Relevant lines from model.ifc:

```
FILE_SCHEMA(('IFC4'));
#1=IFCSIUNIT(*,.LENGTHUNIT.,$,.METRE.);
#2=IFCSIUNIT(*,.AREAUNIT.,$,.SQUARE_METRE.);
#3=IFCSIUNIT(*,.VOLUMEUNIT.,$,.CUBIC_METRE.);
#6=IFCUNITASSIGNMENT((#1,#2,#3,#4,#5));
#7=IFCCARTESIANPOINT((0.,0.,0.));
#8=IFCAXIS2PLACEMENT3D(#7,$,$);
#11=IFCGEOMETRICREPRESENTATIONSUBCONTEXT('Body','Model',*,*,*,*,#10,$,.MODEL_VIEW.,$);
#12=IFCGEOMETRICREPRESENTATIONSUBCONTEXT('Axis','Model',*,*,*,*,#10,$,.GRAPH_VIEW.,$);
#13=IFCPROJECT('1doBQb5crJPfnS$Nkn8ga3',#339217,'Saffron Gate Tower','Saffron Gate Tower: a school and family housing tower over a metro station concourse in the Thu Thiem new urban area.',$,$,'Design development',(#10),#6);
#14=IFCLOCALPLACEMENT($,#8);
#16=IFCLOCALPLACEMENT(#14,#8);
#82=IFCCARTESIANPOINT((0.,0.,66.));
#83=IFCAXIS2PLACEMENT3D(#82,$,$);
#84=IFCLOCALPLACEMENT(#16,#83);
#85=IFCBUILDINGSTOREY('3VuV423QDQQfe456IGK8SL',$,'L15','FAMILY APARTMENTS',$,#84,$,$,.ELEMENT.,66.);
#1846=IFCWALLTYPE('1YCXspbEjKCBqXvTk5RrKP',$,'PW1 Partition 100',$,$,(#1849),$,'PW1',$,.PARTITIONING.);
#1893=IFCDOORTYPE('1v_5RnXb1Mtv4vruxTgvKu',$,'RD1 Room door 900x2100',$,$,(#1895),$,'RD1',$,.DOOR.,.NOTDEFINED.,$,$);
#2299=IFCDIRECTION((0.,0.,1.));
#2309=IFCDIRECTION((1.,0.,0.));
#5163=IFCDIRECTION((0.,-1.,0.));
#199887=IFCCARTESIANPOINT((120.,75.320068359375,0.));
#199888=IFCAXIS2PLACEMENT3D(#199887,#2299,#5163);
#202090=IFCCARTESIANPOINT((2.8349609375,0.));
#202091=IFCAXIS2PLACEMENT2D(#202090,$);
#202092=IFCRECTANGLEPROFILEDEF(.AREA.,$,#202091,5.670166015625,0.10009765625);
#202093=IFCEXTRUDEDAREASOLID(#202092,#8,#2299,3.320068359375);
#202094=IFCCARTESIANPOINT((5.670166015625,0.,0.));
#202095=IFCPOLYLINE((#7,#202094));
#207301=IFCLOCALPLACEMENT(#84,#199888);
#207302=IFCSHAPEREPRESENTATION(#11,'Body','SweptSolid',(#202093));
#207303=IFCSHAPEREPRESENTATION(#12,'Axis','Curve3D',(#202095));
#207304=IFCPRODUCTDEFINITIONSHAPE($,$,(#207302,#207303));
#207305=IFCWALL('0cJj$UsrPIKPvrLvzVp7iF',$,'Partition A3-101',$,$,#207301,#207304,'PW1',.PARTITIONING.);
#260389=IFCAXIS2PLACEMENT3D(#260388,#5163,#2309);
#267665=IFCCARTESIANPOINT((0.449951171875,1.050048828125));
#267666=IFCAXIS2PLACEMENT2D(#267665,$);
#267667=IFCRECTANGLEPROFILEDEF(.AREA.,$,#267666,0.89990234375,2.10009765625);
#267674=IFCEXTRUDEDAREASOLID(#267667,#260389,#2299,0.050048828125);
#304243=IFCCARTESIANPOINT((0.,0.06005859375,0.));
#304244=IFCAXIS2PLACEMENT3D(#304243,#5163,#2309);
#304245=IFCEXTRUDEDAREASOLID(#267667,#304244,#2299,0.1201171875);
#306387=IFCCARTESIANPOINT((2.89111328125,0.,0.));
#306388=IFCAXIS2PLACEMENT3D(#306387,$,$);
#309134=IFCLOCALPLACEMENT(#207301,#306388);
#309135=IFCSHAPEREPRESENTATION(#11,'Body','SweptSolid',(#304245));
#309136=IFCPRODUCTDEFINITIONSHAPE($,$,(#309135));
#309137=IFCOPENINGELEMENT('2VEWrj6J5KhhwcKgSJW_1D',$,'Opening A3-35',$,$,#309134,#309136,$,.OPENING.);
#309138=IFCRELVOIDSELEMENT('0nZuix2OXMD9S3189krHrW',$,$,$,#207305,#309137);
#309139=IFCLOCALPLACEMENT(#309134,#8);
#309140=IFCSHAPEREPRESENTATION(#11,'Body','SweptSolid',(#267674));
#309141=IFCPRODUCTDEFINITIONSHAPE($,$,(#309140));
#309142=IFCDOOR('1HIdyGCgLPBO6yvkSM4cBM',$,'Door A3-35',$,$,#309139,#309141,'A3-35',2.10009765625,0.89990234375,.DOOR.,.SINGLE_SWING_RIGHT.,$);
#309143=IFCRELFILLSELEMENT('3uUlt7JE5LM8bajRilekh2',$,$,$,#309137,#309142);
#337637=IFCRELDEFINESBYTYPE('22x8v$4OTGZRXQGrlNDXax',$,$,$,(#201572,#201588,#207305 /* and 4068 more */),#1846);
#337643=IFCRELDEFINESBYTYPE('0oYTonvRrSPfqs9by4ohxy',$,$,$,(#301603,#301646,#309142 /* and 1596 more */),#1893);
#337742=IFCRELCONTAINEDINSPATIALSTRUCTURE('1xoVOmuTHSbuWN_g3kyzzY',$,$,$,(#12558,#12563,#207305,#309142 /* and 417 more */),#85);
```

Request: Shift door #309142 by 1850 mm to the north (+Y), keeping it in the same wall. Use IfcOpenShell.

```python
import ifcopenshell
import ifcopenshell.api.geometry
import ifcopenshell.util.placement
import ifcopenshell.util.unit

model = ifcopenshell.open("model.ifc")
unit_scale = ifcopenshell.util.unit.calculate_unit_scale(model)

door = model.by_id(309142)
opening = door.FillsVoids[0].RelatingOpeningElement
wall = opening.VoidsElements[0].RelatingBuildingElement

wall_matrix = ifcopenshell.util.placement.get_local_placement(wall.ObjectPlacement)
shift = wall_matrix[:3, 0] * -1.85 / unit_scale
before = ifcopenshell.util.placement.get_local_placement(door.ObjectPlacement)[:3, 3].copy()

# The door is placed relative to its opening, so it follows when the opening moves.
matrix = ifcopenshell.util.placement.get_local_placement(opening.ObjectPlacement)
matrix[:3, 3] += shift
ifcopenshell.api.geometry.edit_object_placement(
    model, product=opening, matrix=matrix, is_si=False, should_transform_children=True
)

after = ifcopenshell.util.placement.get_local_placement(door.ObjectPlacement)[:3, 3]
print("door moved by", (after - before).round(3) + 0.0)

model.write("model_edited.ifc")
```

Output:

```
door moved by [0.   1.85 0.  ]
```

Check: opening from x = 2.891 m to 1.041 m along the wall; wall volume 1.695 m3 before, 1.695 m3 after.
